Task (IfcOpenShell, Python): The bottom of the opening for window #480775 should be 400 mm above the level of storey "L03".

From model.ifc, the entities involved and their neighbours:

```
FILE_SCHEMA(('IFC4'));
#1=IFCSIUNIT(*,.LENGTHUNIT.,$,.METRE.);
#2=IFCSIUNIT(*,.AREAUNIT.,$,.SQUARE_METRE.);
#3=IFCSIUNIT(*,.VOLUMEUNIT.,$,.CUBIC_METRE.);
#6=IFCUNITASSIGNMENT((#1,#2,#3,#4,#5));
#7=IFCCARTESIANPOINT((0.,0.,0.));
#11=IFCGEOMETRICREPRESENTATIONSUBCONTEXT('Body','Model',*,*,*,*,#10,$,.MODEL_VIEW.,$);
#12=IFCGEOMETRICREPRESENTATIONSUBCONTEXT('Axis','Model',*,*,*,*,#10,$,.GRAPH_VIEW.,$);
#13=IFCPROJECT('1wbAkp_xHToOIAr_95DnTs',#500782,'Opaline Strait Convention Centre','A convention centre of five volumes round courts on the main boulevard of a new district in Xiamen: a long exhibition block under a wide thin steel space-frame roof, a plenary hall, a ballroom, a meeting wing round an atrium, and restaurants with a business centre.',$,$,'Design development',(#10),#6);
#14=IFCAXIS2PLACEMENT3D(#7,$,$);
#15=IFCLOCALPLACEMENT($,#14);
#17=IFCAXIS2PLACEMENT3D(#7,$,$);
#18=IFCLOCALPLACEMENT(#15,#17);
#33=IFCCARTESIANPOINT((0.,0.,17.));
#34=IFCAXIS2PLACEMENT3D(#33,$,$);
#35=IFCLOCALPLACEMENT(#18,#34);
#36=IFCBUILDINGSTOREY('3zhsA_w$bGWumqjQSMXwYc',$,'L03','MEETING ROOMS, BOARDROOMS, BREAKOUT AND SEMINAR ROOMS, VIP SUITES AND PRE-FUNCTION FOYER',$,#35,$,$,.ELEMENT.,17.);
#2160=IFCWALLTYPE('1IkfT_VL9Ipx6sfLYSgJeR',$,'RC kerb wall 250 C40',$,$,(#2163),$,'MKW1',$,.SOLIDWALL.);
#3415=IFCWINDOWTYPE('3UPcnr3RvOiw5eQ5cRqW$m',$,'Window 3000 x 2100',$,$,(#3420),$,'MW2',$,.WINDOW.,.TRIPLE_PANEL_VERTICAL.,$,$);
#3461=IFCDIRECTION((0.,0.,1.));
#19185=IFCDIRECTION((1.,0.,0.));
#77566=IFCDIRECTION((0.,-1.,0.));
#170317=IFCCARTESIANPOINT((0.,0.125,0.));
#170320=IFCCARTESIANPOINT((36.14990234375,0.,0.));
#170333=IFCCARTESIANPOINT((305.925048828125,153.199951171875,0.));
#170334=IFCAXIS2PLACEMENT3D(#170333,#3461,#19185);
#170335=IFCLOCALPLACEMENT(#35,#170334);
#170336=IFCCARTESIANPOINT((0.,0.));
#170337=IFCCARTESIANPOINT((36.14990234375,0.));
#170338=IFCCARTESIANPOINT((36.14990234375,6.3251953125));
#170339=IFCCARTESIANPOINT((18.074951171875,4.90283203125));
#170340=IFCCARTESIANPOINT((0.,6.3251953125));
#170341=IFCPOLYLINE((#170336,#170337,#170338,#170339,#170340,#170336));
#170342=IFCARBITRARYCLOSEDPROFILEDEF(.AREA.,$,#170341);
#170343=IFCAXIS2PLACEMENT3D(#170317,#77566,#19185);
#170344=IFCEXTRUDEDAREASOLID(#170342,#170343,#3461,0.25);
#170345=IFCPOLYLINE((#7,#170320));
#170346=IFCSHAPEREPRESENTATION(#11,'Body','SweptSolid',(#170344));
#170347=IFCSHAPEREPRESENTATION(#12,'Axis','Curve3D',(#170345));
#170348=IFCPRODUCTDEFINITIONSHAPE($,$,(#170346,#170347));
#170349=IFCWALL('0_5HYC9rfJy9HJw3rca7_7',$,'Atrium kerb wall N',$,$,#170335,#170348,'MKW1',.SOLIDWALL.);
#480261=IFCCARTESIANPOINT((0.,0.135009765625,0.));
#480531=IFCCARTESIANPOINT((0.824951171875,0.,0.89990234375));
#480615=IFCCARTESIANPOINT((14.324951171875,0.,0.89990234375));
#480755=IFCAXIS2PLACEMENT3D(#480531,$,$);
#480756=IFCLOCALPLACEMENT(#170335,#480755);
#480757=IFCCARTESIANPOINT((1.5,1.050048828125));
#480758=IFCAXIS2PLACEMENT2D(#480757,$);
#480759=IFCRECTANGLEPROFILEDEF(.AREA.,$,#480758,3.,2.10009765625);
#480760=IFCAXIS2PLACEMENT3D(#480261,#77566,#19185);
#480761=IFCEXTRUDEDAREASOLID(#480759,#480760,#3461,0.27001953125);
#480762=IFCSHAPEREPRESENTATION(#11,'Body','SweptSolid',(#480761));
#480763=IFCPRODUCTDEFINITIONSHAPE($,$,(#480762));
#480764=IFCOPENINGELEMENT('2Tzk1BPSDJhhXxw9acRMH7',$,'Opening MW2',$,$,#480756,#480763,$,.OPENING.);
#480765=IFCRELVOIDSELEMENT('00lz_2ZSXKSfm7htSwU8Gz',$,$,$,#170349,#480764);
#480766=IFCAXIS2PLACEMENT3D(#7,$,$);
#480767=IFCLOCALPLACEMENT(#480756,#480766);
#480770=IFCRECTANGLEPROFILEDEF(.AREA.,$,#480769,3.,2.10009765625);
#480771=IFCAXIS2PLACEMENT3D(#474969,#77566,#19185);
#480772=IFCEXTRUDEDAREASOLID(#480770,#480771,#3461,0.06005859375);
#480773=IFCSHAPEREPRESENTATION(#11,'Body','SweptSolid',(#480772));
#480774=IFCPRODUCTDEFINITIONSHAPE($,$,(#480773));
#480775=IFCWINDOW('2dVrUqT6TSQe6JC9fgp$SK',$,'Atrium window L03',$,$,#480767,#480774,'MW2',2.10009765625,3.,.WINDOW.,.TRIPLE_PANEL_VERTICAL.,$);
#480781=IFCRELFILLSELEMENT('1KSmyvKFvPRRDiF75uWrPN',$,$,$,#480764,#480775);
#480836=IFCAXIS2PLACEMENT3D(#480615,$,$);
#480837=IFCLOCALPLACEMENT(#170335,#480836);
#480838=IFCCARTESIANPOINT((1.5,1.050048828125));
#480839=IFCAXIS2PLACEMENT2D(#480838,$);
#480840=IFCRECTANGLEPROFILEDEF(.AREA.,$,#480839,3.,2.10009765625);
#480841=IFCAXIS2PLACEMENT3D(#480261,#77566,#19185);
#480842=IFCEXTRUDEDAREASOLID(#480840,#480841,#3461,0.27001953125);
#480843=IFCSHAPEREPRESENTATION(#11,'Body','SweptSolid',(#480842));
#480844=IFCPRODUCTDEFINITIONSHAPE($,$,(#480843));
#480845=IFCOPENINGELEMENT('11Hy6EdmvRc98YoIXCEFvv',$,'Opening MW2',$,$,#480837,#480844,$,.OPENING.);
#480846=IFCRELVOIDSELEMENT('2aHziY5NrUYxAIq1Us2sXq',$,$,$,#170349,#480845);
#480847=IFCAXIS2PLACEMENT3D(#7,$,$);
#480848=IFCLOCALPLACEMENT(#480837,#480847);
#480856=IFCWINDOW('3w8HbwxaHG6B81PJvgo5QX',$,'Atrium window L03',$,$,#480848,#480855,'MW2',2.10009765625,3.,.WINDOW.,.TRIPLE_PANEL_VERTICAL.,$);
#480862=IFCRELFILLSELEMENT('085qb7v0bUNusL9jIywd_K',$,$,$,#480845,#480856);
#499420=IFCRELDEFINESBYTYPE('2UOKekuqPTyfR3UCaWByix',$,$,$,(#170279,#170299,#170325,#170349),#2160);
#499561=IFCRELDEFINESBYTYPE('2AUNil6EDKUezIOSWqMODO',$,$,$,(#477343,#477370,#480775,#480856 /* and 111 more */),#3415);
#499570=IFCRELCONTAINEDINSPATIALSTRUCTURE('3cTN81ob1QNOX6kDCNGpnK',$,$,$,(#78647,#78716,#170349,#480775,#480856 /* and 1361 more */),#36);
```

```python
import numpy as np
import ifcopenshell
import ifcopenshell.api.geometry
import ifcopenshell.geom
import ifcopenshell.util.element
import ifcopenshell.util.placement
import ifcopenshell.util.shape
import ifcopenshell.util.unit

model = ifcopenshell.open("model.ifc")
unit_scale = ifcopenshell.util.unit.calculate_unit_scale(model)

window = model.by_guid("2dVrUqT6TSQe6JC9fgp$SK")
opening = window.FillsVoids[0].RelatingOpeningElement
storey = ifcopenshell.util.element.get_container(window, ifc_class="IfcBuildingStorey")
level = ifcopenshell.util.placement.get_local_placement(storey.ObjectPlacement)[2, 3]

# The opening's origin need not be at the sill, so measure its lowest point.
shape = ifcopenshell.geom.create_shape(ifcopenshell.geom.settings(), opening)
bottom = ifcopenshell.util.shape.get_shape_bottom_elevation(shape, shape.geometry) / unit_scale
dz = level + 0.4 - bottom

shift = np.array([0.0, 0.0, dz])
# The window is placed relative to its opening, so it follows when the opening moves.
matrix = ifcopenshell.util.placement.get_local_placement(opening.ObjectPlacement)
matrix[:3, 3] += shift
ifcopenshell.api.geometry.edit_object_placement(
    model, product=opening, matrix=matrix, is_si=False, should_transform_children=True
)

print(f"moved by {dz * unit_scale:+.3f} m")

model.write("model_edited.ifc")
```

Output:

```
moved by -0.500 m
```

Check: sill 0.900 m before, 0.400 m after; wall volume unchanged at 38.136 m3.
